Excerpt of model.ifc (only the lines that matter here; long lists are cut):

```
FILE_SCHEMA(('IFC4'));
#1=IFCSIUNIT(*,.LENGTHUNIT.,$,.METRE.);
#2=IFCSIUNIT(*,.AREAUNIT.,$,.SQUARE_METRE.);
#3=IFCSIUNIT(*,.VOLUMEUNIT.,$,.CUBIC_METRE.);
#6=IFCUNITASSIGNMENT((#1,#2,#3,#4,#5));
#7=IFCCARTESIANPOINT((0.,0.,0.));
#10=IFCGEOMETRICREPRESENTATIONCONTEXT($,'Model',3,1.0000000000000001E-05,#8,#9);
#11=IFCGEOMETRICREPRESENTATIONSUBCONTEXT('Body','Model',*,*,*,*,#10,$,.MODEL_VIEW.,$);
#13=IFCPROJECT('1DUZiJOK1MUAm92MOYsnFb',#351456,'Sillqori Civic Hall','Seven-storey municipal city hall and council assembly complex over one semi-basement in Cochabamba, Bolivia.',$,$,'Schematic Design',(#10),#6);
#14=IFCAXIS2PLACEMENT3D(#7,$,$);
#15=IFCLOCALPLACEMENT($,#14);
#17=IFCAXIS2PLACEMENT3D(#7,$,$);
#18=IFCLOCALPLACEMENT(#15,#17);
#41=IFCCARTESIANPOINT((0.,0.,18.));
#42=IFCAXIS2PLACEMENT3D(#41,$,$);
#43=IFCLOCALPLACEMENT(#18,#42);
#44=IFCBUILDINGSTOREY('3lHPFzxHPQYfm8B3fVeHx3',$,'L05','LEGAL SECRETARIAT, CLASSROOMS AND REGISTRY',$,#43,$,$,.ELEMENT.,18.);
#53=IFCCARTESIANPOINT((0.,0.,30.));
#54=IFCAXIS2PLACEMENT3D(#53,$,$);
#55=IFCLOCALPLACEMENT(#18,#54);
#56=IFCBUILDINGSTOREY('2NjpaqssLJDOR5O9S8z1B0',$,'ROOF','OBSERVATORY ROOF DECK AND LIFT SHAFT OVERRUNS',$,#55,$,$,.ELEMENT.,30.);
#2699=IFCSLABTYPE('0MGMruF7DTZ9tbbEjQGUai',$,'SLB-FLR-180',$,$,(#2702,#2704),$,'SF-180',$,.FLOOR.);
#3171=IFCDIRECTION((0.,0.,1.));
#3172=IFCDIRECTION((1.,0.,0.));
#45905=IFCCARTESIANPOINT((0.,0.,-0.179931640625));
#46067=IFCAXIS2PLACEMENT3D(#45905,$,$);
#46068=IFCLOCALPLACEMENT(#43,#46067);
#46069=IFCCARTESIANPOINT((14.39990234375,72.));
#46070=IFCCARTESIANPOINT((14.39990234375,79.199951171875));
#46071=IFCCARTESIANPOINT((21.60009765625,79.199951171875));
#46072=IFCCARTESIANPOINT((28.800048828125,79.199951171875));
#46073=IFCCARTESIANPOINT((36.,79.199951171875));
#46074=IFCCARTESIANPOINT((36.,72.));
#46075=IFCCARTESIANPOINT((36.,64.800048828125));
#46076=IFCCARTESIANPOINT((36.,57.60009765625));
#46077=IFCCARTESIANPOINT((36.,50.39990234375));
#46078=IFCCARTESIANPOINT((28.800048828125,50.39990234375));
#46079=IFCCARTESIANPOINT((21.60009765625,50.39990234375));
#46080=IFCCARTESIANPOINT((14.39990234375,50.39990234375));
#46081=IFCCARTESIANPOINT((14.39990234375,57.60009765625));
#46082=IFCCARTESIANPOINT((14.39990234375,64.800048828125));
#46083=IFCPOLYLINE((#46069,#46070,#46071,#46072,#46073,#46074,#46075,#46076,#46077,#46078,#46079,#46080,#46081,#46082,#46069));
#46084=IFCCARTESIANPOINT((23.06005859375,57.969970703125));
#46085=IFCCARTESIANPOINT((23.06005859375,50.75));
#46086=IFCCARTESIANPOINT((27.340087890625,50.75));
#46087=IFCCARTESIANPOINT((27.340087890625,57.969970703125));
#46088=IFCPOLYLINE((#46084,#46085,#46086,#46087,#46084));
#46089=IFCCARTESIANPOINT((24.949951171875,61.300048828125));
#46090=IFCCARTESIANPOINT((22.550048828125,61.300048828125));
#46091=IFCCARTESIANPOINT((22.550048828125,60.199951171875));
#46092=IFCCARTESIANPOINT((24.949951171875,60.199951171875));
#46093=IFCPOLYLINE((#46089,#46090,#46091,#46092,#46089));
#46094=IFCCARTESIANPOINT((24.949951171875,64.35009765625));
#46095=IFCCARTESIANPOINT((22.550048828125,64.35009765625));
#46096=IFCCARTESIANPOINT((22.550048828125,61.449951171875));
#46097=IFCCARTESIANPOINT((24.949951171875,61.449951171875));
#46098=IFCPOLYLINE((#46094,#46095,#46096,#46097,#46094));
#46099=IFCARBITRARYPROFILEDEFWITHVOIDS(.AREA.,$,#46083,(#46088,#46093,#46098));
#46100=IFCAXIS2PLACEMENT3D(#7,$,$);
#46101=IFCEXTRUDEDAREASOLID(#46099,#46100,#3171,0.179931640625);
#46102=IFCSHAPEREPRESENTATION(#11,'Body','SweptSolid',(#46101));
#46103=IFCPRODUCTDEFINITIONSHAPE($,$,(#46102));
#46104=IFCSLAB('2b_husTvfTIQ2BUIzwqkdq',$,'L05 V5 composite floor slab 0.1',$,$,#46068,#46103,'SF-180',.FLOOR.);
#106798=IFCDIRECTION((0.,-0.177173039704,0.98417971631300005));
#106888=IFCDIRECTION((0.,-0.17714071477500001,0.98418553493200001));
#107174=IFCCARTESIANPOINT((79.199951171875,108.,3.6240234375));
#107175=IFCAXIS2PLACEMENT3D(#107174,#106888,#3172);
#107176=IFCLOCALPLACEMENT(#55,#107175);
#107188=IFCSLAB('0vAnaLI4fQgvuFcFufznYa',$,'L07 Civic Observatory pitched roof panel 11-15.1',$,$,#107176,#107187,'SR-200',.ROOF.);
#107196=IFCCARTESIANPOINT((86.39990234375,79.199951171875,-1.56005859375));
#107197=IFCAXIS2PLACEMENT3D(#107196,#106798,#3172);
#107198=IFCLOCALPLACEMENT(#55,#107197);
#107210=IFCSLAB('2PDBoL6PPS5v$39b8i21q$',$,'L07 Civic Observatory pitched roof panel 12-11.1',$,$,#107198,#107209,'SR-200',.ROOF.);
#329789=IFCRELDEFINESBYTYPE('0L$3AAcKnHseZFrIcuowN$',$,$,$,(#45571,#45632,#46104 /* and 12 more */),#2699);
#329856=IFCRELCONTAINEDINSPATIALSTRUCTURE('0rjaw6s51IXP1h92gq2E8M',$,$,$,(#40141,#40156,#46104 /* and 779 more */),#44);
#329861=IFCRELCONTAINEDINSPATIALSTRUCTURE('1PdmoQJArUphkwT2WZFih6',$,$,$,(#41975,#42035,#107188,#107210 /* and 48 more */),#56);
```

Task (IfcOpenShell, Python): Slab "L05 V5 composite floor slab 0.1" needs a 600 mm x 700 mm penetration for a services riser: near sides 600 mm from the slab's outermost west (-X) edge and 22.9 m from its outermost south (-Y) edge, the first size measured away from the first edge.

```python
import numpy as np
import ifcopenshell
import ifcopenshell.api.feature
import ifcopenshell.api.geometry
import ifcopenshell.api.root
import ifcopenshell.geom
import ifcopenshell.util.placement
import ifcopenshell.util.representation
import ifcopenshell.util.shape
import ifcopenshell.util.unit

model = ifcopenshell.open("model.ifc")
unit_scale = ifcopenshell.util.unit.calculate_unit_scale(model)
settings = ifcopenshell.geom.settings()


def volume(element):
    """Net volume in cubic metres, openings subtracted."""
    shape = ifcopenshell.geom.create_shape(settings, element)
    return ifcopenshell.util.shape.get_volume(shape.geometry)


slab = model.by_id(46104)
before = volume(slab)

# Extent in the slab's own axes, in metres. The edges named are its -X and -Y sides.
slab_shape = ifcopenshell.geom.create_shape(settings, slab)
vertices = ifcopenshell.util.shape.get_vertices(slab_shape.geometry)
x_min, y_min, bottom = vertices.min(axis=0)
top = vertices[:, 2].max()

opening = ifcopenshell.api.root.create_entity(model, ifc_class="IfcOpeningElement", name="Services riser opening", predefined_type="OPENING")
context = ifcopenshell.util.representation.get_context(model, "Model", "Body", "MODEL_VIEW")
width, depth = 0.6, 0.7
outline = [(0.0, 0.0), (width, 0.0), (width, depth), (0.0, depth), (0.0, 0.0)]
# Overshoot both faces by 50 mm so the cut is clean.
shape = ifcopenshell.api.geometry.add_slab_representation(
    model, context=context, depth=top - bottom + 0.1, polyline=outline
)
ifcopenshell.api.geometry.assign_representation(model, product=opening, representation=shape)

matrix = ifcopenshell.util.placement.get_local_placement(slab.ObjectPlacement)
matrix[:, 3] = matrix @ np.append(np.array([x_min + 0.6, y_min + 22.9, bottom - 0.05]) / unit_scale, 1.0)
ifcopenshell.api.geometry.edit_object_placement(model, product=opening, matrix=matrix, is_si=False)
ifcopenshell.api.feature.add_feature(model, feature=opening, element=slab)

after = volume(slab)

print(f"slab volume {before:.3f} -> {after:.3f} m3")

model.write("model_edited.ifc")
```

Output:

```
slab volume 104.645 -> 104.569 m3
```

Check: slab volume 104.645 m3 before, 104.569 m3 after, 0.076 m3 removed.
